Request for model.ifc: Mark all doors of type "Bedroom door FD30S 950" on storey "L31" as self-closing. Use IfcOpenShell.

First a look at what the model holds.

```python
import ifcopenshell
import ifcopenshell.util.element

model = ifcopenshell.open("model.ifc")
print(model.schema)
storey = next(s for s in model.by_type("IfcBuildingStorey") if s.Name == "L31")
doors = [e for e in ifcopenshell.util.element.get_decomposition(storey) if e.is_a("IfcDoor")]
seen = {}
for e in doors:
    element_type = ifcopenshell.util.element.get_type(e)
    key = (element_type.Name if element_type != e and element_type else None, ifcopenshell.util.element.get_pset(e, "Pset_DoorCommon", "SelfClosing"))
    seen[key] = seen.get(key, 0) + 1
for (name, value), count in sorted(seen.items(), key=str):
    print(count, "x", name, "|", value)
```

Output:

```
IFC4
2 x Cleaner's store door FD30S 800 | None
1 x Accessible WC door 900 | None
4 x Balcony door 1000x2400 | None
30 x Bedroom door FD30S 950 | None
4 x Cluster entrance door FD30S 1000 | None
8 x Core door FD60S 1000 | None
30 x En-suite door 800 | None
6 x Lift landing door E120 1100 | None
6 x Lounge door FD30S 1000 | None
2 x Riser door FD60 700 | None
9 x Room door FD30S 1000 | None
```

```python
import ifcopenshell
import ifcopenshell.api.pset
import ifcopenshell.util.element

model = ifcopenshell.open("model.ifc")

storey = next(s for s in model.by_type("IfcBuildingStorey") if s.Name == "L31")
doors = [e for e in ifcopenshell.util.element.get_decomposition(storey) if e.is_a("IfcDoor")]

count = 0
for e in doors:
    element_type = ifcopenshell.util.element.get_type(e)
    if element_type in (None, e) or element_type.Name != "Bedroom door FD30S 950":
        continue
    found = ifcopenshell.util.element.get_pset(e, "Pset_DoorCommon", should_inherit=False)
    if found:
        pset = model.by_id(found["id"])
        if len(ifcopenshell.util.element.get_elements_by_pset(pset)) > 1:
            pset = ifcopenshell.api.pset.unshare_pset(model, products=[e], pset=pset)[0]
    else:
        pset = ifcopenshell.api.pset.add_pset(model, product=e, name="Pset_DoorCommon")
    ifcopenshell.api.pset.edit_pset(model, pset=pset, properties={"SelfClosing": True})
    count += 1

print(count, "doors updated")

model.write("model_edited.ifc")
```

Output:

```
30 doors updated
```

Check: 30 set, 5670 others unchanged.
